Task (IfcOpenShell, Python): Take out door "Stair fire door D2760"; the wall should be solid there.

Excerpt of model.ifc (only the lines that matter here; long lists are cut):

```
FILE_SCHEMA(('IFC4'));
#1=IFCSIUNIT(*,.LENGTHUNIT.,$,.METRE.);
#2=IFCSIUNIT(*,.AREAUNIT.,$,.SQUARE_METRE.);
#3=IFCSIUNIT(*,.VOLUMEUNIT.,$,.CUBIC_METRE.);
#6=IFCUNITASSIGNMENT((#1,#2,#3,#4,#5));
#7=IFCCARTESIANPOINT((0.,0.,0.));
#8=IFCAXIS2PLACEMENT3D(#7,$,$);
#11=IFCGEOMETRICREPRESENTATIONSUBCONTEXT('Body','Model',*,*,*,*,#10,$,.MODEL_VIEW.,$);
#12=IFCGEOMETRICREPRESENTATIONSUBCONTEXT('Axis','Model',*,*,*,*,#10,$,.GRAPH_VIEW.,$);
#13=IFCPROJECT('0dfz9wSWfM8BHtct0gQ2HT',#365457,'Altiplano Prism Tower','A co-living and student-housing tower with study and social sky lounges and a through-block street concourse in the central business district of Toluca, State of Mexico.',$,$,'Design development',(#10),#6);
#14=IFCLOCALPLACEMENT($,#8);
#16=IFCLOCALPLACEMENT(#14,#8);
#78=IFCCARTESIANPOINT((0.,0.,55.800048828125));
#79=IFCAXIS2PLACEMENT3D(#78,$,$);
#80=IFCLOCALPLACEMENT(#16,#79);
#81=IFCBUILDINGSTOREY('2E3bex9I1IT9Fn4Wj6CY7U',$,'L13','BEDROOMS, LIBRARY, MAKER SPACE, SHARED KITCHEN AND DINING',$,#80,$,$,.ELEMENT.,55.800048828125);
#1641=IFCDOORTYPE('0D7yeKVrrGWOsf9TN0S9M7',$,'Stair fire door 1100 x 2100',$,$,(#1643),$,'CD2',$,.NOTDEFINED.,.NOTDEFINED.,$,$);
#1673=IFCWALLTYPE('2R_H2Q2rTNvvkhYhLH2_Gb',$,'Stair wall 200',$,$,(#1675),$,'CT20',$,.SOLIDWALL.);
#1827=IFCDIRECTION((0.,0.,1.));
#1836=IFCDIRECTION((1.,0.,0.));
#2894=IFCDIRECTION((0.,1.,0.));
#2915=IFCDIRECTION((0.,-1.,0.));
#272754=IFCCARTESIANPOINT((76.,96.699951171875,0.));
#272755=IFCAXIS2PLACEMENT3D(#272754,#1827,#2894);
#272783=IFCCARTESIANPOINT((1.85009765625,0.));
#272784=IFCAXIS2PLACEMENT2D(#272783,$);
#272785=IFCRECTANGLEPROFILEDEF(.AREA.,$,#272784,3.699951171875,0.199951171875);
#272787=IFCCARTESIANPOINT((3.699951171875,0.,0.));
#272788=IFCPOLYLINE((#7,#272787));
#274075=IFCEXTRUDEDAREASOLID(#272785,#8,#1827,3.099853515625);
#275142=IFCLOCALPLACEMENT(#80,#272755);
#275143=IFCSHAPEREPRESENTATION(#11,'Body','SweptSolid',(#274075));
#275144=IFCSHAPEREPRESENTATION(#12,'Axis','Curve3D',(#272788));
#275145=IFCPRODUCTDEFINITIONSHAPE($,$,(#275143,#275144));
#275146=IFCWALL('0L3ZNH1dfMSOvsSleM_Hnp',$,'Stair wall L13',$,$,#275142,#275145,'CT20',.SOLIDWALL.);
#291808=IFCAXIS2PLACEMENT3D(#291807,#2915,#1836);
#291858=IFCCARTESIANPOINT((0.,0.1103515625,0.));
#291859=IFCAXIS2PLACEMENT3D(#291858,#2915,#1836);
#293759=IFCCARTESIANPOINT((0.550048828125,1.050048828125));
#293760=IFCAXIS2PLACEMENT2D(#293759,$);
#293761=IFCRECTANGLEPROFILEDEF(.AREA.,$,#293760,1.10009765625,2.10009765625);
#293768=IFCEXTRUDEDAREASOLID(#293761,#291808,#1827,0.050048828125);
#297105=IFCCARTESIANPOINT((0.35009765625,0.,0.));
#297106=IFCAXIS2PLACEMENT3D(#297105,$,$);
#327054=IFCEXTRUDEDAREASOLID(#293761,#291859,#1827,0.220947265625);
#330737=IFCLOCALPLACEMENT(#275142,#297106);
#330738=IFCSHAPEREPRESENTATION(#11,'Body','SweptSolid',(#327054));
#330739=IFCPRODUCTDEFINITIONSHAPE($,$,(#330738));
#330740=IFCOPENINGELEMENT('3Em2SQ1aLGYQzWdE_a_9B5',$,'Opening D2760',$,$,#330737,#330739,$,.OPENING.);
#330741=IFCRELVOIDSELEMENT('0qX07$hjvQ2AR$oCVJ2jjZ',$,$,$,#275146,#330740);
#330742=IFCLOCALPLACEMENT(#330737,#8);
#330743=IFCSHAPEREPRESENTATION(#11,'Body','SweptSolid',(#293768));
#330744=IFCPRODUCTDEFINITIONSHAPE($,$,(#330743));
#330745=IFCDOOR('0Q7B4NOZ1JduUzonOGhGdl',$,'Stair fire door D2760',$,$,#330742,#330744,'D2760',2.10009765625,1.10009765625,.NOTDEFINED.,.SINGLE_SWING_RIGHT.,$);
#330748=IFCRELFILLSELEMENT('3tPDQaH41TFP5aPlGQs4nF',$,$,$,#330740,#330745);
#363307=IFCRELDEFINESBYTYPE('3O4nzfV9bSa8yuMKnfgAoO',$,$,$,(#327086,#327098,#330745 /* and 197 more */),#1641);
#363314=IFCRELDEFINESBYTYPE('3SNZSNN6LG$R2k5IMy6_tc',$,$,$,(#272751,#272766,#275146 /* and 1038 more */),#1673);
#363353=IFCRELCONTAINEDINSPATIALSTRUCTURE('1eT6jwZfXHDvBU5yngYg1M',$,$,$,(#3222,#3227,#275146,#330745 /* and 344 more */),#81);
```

```python
import ifcopenshell
import ifcopenshell.api.feature
import ifcopenshell.api.root
import ifcopenshell.geom
import ifcopenshell.util.shape

model = ifcopenshell.open("model.ifc")
settings = ifcopenshell.geom.settings()


def volume(element):
    """Net volume in cubic metres, openings subtracted."""
    shape = ifcopenshell.geom.create_shape(settings, element)
    return ifcopenshell.util.shape.get_volume(shape.geometry)


door = model.by_id(330745)
opening = door.FillsVoids[0].RelatingOpeningElement
wall = opening.VoidsElements[0].RelatingBuildingElement
before = volume(wall)

ifcopenshell.api.root.remove_product(model, product=door)
ifcopenshell.api.feature.remove_feature(model, feature=opening)

after = volume(wall)

print(f"wall volume {before:.3f} -> {after:.3f} m3")

model.write("model_v2.ifc")
```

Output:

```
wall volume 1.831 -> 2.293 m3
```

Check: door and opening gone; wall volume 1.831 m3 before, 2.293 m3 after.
